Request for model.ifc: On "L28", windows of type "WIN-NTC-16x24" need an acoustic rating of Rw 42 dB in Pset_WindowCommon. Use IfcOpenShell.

First a look at what the model holds.

```python
import ifcopenshell
import ifcopenshell.util.element

model = ifcopenshell.open("model.ifc")
print(model.schema)
storey = next(s for s in model.by_type("IfcBuildingStorey") if s.Name == "L28")
windows = [e for e in ifcopenshell.util.element.get_decomposition(storey) if e.is_a("IfcWindow")]
seen = {}
for e in windows:
    element_type = ifcopenshell.util.element.get_type(e)
    key = (element_type.Name if element_type != e and element_type else None, ifcopenshell.util.element.get_pset(e, "Pset_WindowCommon", "AcousticRating"))
    seen[key] = seen.get(key, 0) + 1
for (name, value), count in sorted(seen.items(), key=str):
    print(count, "x", name, "|", value)
```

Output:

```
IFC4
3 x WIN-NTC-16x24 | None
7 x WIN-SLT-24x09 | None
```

```python
import ifcopenshell
import ifcopenshell.api.pset
import ifcopenshell.util.element

model = ifcopenshell.open("model.ifc")

storey = next(s for s in model.by_type("IfcBuildingStorey") if s.Name == "L28")
windows = [e for e in ifcopenshell.util.element.get_decomposition(storey) if e.is_a("IfcWindow")]

count = 0
for e in windows:
    element_type = ifcopenshell.util.element.get_type(e)
    if element_type in (None, e) or element_type.Name != "WIN-NTC-16x24":
        continue
    found = ifcopenshell.util.element.get_pset(e, "Pset_WindowCommon", should_inherit=False)
    if found:
        pset = model.by_id(found["id"])
        if len(ifcopenshell.util.element.get_elements_by_pset(pset)) > 1:
            pset = ifcopenshell.api.pset.unshare_pset(model, products=[e], pset=pset)[0]
    else:
        pset = ifcopenshell.api.pset.add_pset(model, product=e, name="Pset_WindowCommon")
    ifcopenshell.api.pset.edit_pset(model, pset=pset, properties={"AcousticRating": "Rw 42 dB"})
    count += 1

print(count, "windows updated")

model.write("model_updated.ifc")
```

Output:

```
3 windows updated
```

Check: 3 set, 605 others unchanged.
